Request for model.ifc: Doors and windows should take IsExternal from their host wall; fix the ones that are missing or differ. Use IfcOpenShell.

First a look at what the model holds.

```python
import ifcopenshell
import ifcopenshell.util.element

model = ifcopenshell.open("model.ifc")
print(model.schema)
seen = {}
for e in model.by_type("IfcDoor") + model.by_type("IfcWindow"):
    if not e.FillsVoids:
        continue
    host = e.FillsVoids[0].RelatingOpeningElement.VoidsElements[0].RelatingBuildingElement
    own = ifcopenshell.util.element.get_pset(e, f"Pset_{e.is_a()[3:].removesuffix('StandardCase')}Common", "IsExternal")
    wall = ifcopenshell.util.element.get_pset(host, "Pset_WallCommon", "IsExternal")
    seen[e.is_a(), own, wall] = seen.get((e.is_a(), own, wall), 0) + 1
for (cls, own, wall), count in sorted(seen.items(), key=str):
    print(count, cls, "IsExternal:", own, "| host wall:", wall)
```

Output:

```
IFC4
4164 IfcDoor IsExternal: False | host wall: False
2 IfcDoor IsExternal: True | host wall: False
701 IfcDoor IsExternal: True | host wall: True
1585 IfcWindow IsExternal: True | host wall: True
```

```python
import ifcopenshell
import ifcopenshell.api.pset
import ifcopenshell.util.element

model = ifcopenshell.open("model.ifc")

count = 0
for ifc_class, pset_name in (("IfcDoor", "Pset_DoorCommon"), ("IfcWindow", "Pset_WindowCommon")):
    for e in model.by_type(ifc_class):
        if not e.FillsVoids:
            continue
        host = e.FillsVoids[0].RelatingOpeningElement.VoidsElements[0].RelatingBuildingElement
        external = ifcopenshell.util.element.get_pset(host, "Pset_WallCommon", "IsExternal")
        if external is None or ifcopenshell.util.element.get_pset(e, pset_name, "IsExternal") == external:
            continue
        found = ifcopenshell.util.element.get_pset(e, pset_name, should_inherit=False)
        if found:
            pset = model.by_id(found["id"])
            if len(ifcopenshell.util.element.get_elements_by_pset(pset)) > 1:
                pset = ifcopenshell.api.pset.unshare_pset(model, products=[e], pset=pset)[0]
        else:
            pset = ifcopenshell.api.pset.add_pset(model, product=e, name=pset_name)
        ifcopenshell.api.pset.edit_pset(model, pset=pset, properties={"IsExternal": external})
        count += 1

print(count, "updated")

model.write("model_rev.ifc")
```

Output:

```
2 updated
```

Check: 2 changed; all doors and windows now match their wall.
